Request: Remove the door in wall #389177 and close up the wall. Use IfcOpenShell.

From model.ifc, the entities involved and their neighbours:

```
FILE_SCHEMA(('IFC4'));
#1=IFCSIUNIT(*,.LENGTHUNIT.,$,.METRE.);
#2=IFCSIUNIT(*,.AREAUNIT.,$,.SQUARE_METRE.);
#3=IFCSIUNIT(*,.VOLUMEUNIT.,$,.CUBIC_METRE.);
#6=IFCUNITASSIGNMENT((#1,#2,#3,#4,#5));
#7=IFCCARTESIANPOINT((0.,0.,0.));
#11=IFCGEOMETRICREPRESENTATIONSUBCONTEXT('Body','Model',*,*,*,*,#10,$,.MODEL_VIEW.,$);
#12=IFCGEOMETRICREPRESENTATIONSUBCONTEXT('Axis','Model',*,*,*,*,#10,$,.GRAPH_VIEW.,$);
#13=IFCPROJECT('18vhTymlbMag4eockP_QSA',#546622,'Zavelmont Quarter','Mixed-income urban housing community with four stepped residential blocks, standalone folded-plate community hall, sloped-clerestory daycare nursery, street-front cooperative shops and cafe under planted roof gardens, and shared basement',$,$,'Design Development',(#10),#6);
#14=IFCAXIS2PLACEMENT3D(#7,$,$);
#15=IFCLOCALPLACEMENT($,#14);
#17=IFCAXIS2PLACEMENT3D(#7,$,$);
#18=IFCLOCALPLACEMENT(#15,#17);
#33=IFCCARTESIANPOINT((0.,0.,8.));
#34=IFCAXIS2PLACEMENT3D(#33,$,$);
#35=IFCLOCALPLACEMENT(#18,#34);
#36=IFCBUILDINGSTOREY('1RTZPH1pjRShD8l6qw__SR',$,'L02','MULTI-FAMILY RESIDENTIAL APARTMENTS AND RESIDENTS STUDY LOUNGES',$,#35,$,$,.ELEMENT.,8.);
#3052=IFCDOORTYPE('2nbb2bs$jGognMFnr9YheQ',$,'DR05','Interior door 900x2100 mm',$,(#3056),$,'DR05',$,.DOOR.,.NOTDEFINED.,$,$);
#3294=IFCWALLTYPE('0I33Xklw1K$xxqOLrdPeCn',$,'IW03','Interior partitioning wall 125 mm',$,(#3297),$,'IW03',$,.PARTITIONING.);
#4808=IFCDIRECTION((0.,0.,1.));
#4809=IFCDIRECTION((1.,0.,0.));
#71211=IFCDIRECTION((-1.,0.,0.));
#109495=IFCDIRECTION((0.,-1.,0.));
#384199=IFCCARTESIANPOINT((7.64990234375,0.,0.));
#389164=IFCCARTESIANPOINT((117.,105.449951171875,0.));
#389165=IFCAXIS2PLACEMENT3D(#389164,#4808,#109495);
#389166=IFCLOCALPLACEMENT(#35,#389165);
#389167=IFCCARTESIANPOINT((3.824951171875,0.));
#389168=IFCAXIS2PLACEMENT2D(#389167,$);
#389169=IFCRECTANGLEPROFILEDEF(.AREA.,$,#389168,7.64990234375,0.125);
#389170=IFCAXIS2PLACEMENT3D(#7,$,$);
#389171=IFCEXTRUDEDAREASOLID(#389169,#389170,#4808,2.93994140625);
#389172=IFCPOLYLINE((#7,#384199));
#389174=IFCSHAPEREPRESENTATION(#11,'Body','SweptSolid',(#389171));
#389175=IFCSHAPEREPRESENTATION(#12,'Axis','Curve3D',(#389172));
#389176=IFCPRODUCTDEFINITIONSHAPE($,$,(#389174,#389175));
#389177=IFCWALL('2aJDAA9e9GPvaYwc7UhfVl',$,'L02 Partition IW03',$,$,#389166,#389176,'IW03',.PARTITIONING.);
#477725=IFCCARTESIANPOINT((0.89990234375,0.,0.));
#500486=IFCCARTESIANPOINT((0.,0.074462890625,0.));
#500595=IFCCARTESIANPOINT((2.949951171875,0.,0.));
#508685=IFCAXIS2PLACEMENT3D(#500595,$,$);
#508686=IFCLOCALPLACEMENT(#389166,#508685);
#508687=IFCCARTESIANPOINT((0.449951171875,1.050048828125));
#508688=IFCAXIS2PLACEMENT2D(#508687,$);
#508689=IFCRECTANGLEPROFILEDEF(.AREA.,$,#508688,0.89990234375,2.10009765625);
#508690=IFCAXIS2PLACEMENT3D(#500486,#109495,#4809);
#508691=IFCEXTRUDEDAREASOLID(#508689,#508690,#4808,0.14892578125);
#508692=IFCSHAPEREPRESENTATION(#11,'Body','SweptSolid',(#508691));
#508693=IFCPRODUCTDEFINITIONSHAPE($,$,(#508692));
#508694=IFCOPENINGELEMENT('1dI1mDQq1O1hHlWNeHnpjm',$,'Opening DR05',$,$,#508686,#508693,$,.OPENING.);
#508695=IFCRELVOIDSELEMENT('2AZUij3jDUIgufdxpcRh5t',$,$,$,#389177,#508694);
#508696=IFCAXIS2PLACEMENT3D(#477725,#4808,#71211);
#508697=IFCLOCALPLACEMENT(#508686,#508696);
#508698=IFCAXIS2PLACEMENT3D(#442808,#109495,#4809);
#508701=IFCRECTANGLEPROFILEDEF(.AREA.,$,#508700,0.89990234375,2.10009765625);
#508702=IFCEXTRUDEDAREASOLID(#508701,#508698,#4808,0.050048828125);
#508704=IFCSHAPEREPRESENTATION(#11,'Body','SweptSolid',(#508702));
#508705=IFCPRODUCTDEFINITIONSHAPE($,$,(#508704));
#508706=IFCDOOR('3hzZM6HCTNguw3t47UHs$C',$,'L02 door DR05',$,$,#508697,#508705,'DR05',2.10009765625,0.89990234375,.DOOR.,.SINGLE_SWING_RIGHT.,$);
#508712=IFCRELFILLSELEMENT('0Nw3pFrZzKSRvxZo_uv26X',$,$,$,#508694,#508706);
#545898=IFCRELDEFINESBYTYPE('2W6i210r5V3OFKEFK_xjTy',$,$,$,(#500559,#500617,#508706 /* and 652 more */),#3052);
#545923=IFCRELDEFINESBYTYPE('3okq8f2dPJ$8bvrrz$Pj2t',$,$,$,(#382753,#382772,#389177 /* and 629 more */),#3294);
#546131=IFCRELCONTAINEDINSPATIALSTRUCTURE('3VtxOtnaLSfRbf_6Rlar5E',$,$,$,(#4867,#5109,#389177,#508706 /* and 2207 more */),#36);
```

```python
import ifcopenshell
import ifcopenshell.api.feature
import ifcopenshell.api.root
import ifcopenshell.geom
import ifcopenshell.util.shape

model = ifcopenshell.open("model.ifc")
settings = ifcopenshell.geom.settings()


def volume(element):
    """Net volume in cubic metres, openings subtracted."""
    shape = ifcopenshell.geom.create_shape(settings, element)
    return ifcopenshell.util.shape.get_volume(shape.geometry)


door = model.by_guid("3hzZM6HCTNguw3t47UHs$C")
opening = door.FillsVoids[0].RelatingOpeningElement
wall = opening.VoidsElements[0].RelatingBuildingElement
before = volume(wall)

ifcopenshell.api.root.remove_product(model, product=door)
ifcopenshell.api.feature.remove_feature(model, feature=opening)

after = volume(wall)

print(f"wall volume {before:.3f} -> {after:.3f} m3")

model.write("model_updated.ifc")
```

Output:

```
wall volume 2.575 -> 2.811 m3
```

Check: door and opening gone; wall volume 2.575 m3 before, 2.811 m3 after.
